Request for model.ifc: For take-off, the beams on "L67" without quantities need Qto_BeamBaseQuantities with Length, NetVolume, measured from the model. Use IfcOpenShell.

First a look at what the model holds.

```python
import ifcopenshell
import ifcopenshell.util.element
import ifcopenshell.util.unit

model = ifcopenshell.open("model.ifc")
print(model.schema)
for unit_type in ("LENGTHUNIT", "AREAUNIT", "VOLUMEUNIT"):
    print(unit_type, ifcopenshell.util.unit.calculate_unit_scale(model, unit_type))
storey = next(s for s in model.by_type("IfcBuildingStorey") if s.Name == "L67")
beams = [e for e in ifcopenshell.util.element.get_decomposition(storey) if e.is_a("IfcBeam")]
for e in sorted(beams, key=lambda e: e.id()):
    print(e.id(), e.is_a(), e.Name, list(ifcopenshell.util.element.get_psets(e, qtos_only=True)), sep=" | ")
```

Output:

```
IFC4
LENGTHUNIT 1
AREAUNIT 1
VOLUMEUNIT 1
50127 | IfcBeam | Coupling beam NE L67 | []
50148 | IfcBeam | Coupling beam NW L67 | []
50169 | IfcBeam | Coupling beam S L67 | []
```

```python
import ifcopenshell
import ifcopenshell.api.pset
import ifcopenshell.geom
import ifcopenshell.util.element
import ifcopenshell.util.shape
import ifcopenshell.util.unit

model = ifcopenshell.open("model.ifc")
unit_scale = ifcopenshell.util.unit.calculate_unit_scale(model)
volume_scale = ifcopenshell.util.unit.calculate_unit_scale(model, "VOLUMEUNIT")
settings = ifcopenshell.geom.settings()

storey = next(s for s in model.by_type("IfcBuildingStorey") if s.Name == "L67")
beams = [e for e in ifcopenshell.util.element.get_decomposition(storey) if e.is_a("IfcBeam")]

for e in sorted(beams, key=lambda e: e.id()):
    if ifcopenshell.util.element.get_psets(e, qtos_only=True, should_inherit=False):
        continue
    # Geometry comes back in metres, in the element's own axes.
    shape = ifcopenshell.geom.create_shape(settings, e)
    values = {
        "Length": ifcopenshell.util.shape.get_max_xyz(shape.geometry) / unit_scale,
        "NetVolume": ifcopenshell.util.shape.get_volume(shape.geometry) / volume_scale,
    }
    qto = ifcopenshell.api.pset.add_qto(model, product=e, name="Qto_BeamBaseQuantities")
    ifcopenshell.api.pset.edit_qto(model, qto=qto, properties=values)
    print(e.id(), {k: round(v, 3) for k, v in values.items()})

model.write("model-out.ifc")
```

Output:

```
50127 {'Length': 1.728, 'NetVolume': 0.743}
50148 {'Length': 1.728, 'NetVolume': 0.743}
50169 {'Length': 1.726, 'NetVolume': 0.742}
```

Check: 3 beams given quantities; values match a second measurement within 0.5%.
